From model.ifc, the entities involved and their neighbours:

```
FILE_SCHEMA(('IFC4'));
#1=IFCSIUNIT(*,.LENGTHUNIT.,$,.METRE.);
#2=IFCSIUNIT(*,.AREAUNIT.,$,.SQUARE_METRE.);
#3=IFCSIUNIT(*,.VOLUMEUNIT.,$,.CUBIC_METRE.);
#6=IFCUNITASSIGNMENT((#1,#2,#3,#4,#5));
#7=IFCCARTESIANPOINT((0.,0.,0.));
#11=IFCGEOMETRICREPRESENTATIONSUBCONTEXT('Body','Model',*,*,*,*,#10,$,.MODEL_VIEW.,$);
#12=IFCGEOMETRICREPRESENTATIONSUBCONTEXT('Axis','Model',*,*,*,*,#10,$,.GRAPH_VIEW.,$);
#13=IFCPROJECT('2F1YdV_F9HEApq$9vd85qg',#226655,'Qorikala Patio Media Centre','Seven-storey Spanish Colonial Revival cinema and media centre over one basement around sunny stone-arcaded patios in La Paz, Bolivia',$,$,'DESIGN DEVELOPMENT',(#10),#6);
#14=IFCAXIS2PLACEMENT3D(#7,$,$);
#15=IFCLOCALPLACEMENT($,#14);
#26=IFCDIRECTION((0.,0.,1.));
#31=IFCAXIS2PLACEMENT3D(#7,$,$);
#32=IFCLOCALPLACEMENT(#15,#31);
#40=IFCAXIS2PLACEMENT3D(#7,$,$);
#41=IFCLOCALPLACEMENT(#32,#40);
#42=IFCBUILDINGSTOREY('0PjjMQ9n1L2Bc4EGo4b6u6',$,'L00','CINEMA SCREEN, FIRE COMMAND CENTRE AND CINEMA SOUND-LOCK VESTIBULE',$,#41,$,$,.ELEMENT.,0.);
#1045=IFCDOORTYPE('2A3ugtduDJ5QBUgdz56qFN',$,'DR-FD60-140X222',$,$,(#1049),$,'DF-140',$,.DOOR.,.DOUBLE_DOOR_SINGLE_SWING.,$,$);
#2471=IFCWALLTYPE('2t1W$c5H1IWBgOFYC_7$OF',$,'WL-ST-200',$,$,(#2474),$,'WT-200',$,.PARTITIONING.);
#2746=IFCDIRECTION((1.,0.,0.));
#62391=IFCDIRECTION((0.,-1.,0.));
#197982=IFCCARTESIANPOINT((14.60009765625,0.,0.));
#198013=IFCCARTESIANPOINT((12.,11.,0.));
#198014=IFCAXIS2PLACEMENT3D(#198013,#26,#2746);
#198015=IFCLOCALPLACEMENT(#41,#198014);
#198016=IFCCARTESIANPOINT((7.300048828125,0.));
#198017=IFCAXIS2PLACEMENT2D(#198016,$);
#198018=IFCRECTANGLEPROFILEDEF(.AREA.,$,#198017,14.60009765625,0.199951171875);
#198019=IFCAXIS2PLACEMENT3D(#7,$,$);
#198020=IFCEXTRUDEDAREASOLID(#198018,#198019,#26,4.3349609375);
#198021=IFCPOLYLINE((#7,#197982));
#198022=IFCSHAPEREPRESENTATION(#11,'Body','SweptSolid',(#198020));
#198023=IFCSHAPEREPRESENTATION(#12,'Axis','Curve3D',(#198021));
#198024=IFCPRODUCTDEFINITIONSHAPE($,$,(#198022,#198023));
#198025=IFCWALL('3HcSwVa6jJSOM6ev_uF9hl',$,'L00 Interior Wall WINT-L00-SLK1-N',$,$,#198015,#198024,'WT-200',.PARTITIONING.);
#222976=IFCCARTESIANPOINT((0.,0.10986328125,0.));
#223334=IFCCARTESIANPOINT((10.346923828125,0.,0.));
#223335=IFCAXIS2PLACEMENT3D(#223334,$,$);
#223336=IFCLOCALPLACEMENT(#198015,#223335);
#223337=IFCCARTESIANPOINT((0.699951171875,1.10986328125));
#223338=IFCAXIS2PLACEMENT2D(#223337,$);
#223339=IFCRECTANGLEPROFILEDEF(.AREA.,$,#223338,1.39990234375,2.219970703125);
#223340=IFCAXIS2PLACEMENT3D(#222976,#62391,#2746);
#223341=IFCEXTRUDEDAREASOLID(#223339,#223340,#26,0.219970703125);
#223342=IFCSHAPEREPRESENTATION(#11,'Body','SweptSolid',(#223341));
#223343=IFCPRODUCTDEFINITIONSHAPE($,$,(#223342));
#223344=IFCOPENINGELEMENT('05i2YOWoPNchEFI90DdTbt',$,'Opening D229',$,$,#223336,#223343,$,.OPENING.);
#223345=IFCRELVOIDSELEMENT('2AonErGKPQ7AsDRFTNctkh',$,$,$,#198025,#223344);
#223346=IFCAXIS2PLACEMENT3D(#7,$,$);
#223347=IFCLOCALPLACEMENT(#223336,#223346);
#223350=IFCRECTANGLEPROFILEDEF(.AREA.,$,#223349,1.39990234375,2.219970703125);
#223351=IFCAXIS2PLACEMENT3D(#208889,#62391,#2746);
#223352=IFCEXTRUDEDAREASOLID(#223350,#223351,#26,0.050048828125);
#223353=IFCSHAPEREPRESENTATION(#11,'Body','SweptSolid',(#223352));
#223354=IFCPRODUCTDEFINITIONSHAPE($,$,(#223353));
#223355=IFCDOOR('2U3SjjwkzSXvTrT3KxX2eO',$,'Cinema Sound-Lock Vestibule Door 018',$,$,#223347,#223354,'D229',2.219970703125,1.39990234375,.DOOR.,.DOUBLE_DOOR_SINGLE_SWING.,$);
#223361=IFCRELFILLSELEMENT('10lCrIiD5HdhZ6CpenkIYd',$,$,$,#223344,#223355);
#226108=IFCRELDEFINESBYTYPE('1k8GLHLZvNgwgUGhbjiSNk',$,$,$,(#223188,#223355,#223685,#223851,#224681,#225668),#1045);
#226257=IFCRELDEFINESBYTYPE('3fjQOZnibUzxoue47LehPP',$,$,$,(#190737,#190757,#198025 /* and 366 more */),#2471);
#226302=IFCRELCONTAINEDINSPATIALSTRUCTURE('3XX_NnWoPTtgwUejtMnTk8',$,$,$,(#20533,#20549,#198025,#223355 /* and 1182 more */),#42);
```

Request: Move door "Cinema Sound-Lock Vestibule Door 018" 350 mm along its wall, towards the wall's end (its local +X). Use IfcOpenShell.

```python
import ifcopenshell
import ifcopenshell.api.geometry
import ifcopenshell.util.placement

model = ifcopenshell.open("model.ifc")

door = model.by_id(223355)
opening = door.FillsVoids[0].RelatingOpeningElement
wall = opening.VoidsElements[0].RelatingBuildingElement

wall_matrix = ifcopenshell.util.placement.get_local_placement(wall.ObjectPlacement)
shift = wall_matrix[:3, 0] * 0.35
before = ifcopenshell.util.placement.get_local_placement(door.ObjectPlacement)[:3, 3].copy()

# The door is placed relative to its opening, so it follows when the opening moves.
matrix = ifcopenshell.util.placement.get_local_placement(opening.ObjectPlacement)
matrix[:3, 3] += shift
ifcopenshell.api.geometry.edit_object_placement(
    model, product=opening, matrix=matrix, is_si=False, should_transform_children=True
)

after = ifcopenshell.util.placement.get_local_placement(door.ObjectPlacement)[:3, 3]
print("door moved by", (after - before).round(3) + 0.0)

model.write("model_updated.ifc")
```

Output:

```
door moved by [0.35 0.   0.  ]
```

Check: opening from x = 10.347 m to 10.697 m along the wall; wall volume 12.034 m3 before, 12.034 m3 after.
